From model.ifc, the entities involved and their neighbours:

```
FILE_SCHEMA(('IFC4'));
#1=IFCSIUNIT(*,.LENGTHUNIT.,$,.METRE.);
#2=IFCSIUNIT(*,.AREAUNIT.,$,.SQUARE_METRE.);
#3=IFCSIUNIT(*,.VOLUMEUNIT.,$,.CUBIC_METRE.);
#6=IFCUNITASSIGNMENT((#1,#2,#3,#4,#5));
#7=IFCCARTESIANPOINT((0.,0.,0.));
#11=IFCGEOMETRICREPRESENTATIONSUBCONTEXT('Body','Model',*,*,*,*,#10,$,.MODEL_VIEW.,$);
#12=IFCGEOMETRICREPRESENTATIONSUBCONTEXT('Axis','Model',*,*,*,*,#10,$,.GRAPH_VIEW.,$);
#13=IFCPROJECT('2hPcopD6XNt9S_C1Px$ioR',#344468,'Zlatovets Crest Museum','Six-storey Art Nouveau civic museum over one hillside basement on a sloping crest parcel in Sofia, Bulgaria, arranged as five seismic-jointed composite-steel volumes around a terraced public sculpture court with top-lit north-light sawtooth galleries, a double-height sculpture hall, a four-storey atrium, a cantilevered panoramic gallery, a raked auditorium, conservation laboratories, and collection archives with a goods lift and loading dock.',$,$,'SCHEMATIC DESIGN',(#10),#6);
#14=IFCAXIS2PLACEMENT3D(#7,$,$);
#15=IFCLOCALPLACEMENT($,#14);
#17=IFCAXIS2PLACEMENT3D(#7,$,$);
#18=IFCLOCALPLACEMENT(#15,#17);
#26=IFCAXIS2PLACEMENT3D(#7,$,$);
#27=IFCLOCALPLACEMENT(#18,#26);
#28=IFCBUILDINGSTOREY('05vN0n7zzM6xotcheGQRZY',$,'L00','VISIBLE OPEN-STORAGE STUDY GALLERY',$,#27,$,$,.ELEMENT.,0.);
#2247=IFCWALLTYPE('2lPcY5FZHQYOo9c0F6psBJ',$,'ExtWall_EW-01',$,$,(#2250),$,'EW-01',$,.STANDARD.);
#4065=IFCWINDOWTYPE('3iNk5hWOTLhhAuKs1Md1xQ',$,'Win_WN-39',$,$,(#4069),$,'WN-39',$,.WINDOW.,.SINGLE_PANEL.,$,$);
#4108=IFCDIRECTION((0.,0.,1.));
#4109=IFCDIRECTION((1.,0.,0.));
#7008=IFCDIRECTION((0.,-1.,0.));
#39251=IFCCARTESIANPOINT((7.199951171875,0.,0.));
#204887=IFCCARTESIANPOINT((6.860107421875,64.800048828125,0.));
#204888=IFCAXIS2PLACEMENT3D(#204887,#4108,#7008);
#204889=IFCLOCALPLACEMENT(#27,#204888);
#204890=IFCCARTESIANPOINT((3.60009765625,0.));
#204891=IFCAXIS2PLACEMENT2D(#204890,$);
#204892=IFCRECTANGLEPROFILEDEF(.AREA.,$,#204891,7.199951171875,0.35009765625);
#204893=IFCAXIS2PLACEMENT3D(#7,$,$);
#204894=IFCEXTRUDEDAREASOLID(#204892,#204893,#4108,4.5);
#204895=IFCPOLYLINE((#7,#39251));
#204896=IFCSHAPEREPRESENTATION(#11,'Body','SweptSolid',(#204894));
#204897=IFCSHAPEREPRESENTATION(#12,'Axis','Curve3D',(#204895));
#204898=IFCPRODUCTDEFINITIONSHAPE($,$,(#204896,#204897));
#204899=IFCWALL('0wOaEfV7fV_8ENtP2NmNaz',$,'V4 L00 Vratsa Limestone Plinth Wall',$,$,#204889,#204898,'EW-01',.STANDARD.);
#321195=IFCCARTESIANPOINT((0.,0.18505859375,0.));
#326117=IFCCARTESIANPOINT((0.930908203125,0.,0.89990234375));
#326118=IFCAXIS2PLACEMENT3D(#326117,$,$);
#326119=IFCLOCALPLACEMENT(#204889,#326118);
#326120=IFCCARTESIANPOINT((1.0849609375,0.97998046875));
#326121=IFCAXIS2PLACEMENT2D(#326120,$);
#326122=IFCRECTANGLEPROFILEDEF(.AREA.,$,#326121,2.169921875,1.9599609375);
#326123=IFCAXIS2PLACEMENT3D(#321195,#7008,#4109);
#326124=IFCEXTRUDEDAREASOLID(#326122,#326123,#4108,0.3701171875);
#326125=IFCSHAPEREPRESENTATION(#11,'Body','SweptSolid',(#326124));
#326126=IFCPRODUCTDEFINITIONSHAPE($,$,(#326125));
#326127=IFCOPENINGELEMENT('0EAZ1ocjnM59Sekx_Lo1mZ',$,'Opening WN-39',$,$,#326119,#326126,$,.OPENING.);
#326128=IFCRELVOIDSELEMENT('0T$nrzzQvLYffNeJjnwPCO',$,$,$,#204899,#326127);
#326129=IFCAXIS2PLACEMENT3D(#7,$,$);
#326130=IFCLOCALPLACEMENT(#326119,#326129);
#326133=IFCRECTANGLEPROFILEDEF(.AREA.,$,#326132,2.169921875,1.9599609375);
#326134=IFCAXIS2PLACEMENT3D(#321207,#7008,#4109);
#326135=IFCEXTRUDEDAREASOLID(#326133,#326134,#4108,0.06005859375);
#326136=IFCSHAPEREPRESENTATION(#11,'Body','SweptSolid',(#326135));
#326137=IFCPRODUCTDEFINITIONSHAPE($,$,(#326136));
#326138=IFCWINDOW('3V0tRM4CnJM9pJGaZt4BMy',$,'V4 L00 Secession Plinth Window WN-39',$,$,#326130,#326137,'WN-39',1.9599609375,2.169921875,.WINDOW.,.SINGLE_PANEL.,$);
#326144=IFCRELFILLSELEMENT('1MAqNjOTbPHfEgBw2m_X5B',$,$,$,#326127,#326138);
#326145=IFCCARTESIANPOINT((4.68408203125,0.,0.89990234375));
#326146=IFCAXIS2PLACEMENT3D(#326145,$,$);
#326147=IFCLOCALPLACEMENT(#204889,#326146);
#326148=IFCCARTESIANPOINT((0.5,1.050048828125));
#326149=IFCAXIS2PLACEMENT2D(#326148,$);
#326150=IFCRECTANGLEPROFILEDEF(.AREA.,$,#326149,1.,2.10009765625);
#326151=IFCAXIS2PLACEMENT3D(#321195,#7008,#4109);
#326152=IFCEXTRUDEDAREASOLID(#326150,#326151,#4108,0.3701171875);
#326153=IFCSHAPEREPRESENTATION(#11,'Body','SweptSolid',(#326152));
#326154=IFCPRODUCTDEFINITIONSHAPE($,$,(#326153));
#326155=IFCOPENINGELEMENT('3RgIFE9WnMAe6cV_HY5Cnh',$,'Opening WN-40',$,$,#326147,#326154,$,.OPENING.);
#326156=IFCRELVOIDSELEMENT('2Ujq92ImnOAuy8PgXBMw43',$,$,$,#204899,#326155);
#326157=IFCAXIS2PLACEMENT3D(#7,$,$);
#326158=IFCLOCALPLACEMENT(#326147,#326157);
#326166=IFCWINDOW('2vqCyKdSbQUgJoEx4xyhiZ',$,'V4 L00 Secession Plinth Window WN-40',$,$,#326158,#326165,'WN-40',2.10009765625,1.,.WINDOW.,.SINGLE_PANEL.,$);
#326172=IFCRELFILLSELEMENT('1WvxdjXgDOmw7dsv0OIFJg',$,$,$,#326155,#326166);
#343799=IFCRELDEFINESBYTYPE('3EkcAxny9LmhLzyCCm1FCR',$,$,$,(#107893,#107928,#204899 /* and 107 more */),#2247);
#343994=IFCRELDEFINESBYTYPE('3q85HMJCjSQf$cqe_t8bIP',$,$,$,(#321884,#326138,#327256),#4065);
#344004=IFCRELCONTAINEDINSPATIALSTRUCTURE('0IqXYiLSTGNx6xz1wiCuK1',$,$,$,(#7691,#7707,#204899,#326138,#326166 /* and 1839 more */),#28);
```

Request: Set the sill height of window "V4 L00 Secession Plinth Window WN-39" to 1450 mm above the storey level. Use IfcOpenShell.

```python
import numpy as np
import ifcopenshell
import ifcopenshell.api.geometry
import ifcopenshell.geom
import ifcopenshell.util.element
import ifcopenshell.util.placement
import ifcopenshell.util.shape
import ifcopenshell.util.unit

model = ifcopenshell.open("model.ifc")
unit_scale = ifcopenshell.util.unit.calculate_unit_scale(model)

window = model.by_guid("3V0tRM4CnJM9pJGaZt4BMy")
opening = window.FillsVoids[0].RelatingOpeningElement
storey = ifcopenshell.util.element.get_container(window, ifc_class="IfcBuildingStorey")
level = ifcopenshell.util.placement.get_local_placement(storey.ObjectPlacement)[2, 3]

# The opening's origin need not be at the sill, so measure its lowest point.
shape = ifcopenshell.geom.create_shape(ifcopenshell.geom.settings(), opening)
bottom = ifcopenshell.util.shape.get_shape_bottom_elevation(shape, shape.geometry) / unit_scale
dz = level + 1.45 / unit_scale - bottom

shift = np.array([0.0, 0.0, dz])
# The window is placed relative to its opening, so it follows when the opening moves.
matrix = ifcopenshell.util.placement.get_local_placement(opening.ObjectPlacement)
matrix[:3, 3] += shift
ifcopenshell.api.geometry.edit_object_placement(
    model, product=opening, matrix=matrix, is_si=False, should_transform_children=True
)

print(f"moved by {dz * unit_scale:+.3f} m")

model.write("model_updated.ifc")
```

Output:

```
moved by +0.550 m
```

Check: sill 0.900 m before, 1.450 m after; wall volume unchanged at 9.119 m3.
